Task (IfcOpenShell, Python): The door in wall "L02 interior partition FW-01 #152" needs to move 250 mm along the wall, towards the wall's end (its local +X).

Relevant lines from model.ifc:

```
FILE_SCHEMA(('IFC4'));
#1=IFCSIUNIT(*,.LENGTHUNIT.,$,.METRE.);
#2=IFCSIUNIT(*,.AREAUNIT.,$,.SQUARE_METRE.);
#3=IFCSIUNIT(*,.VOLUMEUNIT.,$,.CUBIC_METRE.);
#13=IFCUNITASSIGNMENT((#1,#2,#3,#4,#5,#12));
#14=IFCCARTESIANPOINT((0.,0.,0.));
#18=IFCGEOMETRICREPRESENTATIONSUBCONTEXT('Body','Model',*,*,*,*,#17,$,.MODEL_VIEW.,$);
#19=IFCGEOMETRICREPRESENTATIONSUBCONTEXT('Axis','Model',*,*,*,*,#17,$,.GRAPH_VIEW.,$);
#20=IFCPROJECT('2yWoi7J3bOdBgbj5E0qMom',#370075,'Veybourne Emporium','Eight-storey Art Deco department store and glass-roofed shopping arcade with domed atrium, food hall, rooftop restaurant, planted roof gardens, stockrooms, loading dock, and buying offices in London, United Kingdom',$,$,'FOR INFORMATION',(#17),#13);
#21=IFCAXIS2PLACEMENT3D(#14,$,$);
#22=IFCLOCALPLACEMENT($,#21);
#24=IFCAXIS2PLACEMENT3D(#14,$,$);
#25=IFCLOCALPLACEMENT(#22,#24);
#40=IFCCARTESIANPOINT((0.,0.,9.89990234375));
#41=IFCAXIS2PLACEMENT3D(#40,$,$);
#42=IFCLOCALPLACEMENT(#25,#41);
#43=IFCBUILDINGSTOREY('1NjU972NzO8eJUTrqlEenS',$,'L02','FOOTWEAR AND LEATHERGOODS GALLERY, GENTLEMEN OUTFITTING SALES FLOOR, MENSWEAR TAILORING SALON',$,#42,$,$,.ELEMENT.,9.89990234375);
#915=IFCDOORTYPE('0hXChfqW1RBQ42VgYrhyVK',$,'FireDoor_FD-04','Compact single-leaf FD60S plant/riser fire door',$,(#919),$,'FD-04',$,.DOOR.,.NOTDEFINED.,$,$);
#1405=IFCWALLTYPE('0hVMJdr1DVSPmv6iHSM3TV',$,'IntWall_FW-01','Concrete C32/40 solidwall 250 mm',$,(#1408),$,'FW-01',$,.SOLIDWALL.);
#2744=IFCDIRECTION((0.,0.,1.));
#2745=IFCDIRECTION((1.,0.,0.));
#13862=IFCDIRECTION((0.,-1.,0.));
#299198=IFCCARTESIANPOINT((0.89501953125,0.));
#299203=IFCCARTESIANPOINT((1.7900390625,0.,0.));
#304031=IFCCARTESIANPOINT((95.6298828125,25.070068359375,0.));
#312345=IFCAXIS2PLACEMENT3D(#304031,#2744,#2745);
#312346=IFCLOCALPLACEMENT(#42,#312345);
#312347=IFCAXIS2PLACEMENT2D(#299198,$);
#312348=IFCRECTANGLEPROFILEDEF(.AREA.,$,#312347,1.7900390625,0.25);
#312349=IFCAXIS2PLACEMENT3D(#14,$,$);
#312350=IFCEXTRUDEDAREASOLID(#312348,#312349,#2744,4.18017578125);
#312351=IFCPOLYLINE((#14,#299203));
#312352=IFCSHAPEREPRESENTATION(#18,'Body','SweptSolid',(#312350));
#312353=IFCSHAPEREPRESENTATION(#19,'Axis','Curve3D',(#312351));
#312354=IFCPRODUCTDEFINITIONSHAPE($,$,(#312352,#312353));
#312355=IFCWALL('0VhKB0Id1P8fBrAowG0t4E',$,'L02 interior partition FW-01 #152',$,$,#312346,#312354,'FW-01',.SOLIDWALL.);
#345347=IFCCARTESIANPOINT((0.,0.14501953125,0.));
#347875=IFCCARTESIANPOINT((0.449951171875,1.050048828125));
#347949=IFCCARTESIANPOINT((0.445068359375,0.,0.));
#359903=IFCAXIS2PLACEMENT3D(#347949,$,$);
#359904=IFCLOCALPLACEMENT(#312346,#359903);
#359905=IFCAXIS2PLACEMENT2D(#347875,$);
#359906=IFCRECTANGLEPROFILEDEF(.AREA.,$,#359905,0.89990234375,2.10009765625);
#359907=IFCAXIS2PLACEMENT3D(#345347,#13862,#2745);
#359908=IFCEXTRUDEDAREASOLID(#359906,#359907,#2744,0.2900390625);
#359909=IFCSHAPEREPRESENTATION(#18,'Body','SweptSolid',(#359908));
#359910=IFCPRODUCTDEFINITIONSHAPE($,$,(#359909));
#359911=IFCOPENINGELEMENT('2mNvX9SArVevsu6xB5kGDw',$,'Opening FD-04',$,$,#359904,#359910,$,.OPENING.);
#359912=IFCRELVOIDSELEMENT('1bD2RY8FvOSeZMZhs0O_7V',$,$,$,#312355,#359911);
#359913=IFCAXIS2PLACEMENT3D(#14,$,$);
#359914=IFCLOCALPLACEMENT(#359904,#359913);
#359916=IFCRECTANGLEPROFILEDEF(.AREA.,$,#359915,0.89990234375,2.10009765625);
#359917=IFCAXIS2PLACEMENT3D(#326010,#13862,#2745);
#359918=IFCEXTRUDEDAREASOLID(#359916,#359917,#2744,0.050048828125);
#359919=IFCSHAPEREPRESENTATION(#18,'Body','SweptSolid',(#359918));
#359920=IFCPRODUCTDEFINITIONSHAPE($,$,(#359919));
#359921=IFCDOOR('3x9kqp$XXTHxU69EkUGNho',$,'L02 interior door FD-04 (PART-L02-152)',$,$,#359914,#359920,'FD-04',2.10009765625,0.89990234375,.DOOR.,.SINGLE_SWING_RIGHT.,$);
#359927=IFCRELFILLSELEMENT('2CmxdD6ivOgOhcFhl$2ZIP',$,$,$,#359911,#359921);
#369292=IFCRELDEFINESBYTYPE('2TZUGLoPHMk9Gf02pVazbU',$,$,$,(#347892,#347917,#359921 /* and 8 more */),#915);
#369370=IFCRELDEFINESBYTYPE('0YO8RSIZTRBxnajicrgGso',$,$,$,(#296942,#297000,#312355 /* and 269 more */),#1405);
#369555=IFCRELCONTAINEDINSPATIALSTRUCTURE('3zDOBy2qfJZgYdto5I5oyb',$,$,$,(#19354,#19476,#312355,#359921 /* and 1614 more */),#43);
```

```python
import ifcopenshell
import ifcopenshell.api.geometry
import ifcopenshell.util.placement
import ifcopenshell.util.unit

model = ifcopenshell.open("model.ifc")
unit_scale = ifcopenshell.util.unit.calculate_unit_scale(model)

door = model.by_id(359921)
opening = door.FillsVoids[0].RelatingOpeningElement
wall = opening.VoidsElements[0].RelatingBuildingElement

wall_matrix = ifcopenshell.util.placement.get_local_placement(wall.ObjectPlacement)
shift = wall_matrix[:3, 0] * 0.25 / unit_scale
before = ifcopenshell.util.placement.get_local_placement(door.ObjectPlacement)[:3, 3].copy()

# The door is placed relative to its opening, so it follows when the opening moves.
matrix = ifcopenshell.util.placement.get_local_placement(opening.ObjectPlacement)
matrix[:3, 3] += shift
ifcopenshell.api.geometry.edit_object_placement(
    model, product=opening, matrix=matrix, is_si=False, should_transform_children=True
)

after = ifcopenshell.util.placement.get_local_placement(door.ObjectPlacement)[:3, 3]
print("door moved by", (after - before).round(3) + 0.0)

model.write("model_v2.ifc")
```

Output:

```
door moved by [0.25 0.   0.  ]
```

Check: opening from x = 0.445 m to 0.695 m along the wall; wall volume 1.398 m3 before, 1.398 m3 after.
